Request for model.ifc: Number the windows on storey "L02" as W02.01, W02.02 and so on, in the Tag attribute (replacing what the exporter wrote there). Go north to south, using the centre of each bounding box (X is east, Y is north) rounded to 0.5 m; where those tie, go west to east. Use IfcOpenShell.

First a look at what the model holds.

```python
import ifcopenshell
import ifcopenshell.util.element
import ifcopenshell.util.placement

model = ifcopenshell.open("model.ifc")
print(model.schema)
storey = next(s for s in model.by_type("IfcBuildingStorey") if s.Name == "L02")
windows = [e for e in ifcopenshell.util.element.get_decomposition(storey) if e.is_a("IfcWindow")]
for e in sorted(windows, key=lambda e: e.id()):
    origin = ifcopenshell.util.placement.get_local_placement(e.ObjectPlacement)[:3, 3]
    print(e.id(), e.Tag, e.Name, origin.round(2) + 0.0, sep=" | ")
```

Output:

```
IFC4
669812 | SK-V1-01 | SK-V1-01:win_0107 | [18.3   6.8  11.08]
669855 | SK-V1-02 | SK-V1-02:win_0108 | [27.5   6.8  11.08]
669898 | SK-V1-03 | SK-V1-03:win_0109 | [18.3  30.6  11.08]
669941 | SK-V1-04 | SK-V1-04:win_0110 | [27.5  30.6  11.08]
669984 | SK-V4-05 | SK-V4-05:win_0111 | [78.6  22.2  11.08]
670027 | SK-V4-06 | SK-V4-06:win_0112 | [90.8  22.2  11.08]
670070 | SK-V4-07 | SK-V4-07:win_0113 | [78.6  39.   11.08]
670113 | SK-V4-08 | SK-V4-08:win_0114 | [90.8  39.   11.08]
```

```python
import ifcopenshell
import ifcopenshell.geom
import ifcopenshell.util.element
import ifcopenshell.util.shape

model = ifcopenshell.open("model.ifc")
settings = ifcopenshell.geom.settings()
settings.set("use-world-coords", True)


def centre(element):
    shape = ifcopenshell.geom.create_shape(settings, element)
    return ifcopenshell.util.shape.get_bbox_centroid(shape.geometry)


storey = next(s for s in model.by_type("IfcBuildingStorey") if s.Name == "L02")
windows = [e for e in ifcopenshell.util.element.get_decomposition(storey) if e.is_a("IfcWindow")]

# Insertion points can sit at a corner or the storey origin, so sort by the geometry (in metres).
centres = {e: centre(e) for e in windows}
windows.sort(key=lambda e: (-round(centres[e][1] / 0.5), centres[e][0]))

for i, e in enumerate(windows, start=1):
    number = f"W02.{i:02d}"
    e.Tag = number
    print(e.id(), number)

model.write("model_v2.ifc")
```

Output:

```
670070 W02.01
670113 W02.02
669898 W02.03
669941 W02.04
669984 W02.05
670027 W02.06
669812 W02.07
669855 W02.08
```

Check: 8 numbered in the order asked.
